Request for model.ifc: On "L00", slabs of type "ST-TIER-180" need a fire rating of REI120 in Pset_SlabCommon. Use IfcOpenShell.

First a look at what the model holds.

```python
import ifcopenshell
import ifcopenshell.util.element

model = ifcopenshell.open("model.ifc")
print(model.schema)
storey = next(s for s in model.by_type("IfcBuildingStorey") if s.Name == "L00")
slabs = [e for e in ifcopenshell.util.element.get_decomposition(storey) if e.is_a("IfcSlab")]
seen = {}
for e in slabs:
    element_type = ifcopenshell.util.element.get_type(e)
    key = (element_type.Name if element_type != e and element_type else None, ifcopenshell.util.element.get_pset(e, "Pset_SlabCommon", "FireRating"))
    seen[key] = seen.get(key, 0) + 1
for (name, value), count in sorted(seen.items(), key=str):
    print(count, "x", name, "|", value)
```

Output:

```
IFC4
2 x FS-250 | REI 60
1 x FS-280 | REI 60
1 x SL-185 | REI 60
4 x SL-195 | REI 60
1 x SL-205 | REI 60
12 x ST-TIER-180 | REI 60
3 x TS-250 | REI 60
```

```python
import ifcopenshell
import ifcopenshell.api.pset
import ifcopenshell.util.element

model = ifcopenshell.open("model.ifc")

storey = next(s for s in model.by_type("IfcBuildingStorey") if s.Name == "L00")
slabs = [e for e in ifcopenshell.util.element.get_decomposition(storey) if e.is_a("IfcSlab")]

count = 0
for e in slabs:
    element_type = ifcopenshell.util.element.get_type(e)
    if element_type in (None, e) or element_type.Name != "ST-TIER-180":
        continue
    # add_pset returns the element's existing set when there is one.
    pset = ifcopenshell.api.pset.add_pset(model, product=e, name="Pset_SlabCommon")
    ifcopenshell.api.pset.edit_pset(model, pset=pset, properties={"FireRating": "REI120"})
    count += 1

print(count, "slabs updated")

model.write("model_v2.ifc")
```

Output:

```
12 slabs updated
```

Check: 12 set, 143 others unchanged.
